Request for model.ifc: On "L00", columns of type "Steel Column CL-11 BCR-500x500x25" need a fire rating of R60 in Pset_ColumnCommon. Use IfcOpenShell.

First a look at what the model holds.

```python
import ifcopenshell
import ifcopenshell.util.element

model = ifcopenshell.open("model.ifc")
print(model.schema)
storey = next(s for s in model.by_type("IfcBuildingStorey") if s.Name == "L00")
columns = [e for e in ifcopenshell.util.element.get_decomposition(storey) if e.is_a("IfcColumn")]
seen = {}
for e in columns:
    element_type = ifcopenshell.util.element.get_type(e)
    key = (element_type.Name if element_type != e and element_type else None, ifcopenshell.util.element.get_pset(e, "Pset_ColumnCommon", "FireRating"))
    seen[key] = seen.get(key, 0) + 1
for (name, value), count in sorted(seen.items(), key=str):
    print(count, "x", name, "|", value)
```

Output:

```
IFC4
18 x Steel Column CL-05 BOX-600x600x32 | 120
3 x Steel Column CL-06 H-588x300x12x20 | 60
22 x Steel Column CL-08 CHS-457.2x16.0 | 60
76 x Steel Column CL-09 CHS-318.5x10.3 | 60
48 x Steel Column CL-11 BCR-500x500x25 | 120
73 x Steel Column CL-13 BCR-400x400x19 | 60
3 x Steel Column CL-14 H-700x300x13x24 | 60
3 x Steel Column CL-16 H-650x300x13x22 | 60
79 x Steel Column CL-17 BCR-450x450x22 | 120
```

```python
import ifcopenshell
import ifcopenshell.api.pset
import ifcopenshell.util.element

model = ifcopenshell.open("model.ifc")

storey = next(s for s in model.by_type("IfcBuildingStorey") if s.Name == "L00")
columns = [e for e in ifcopenshell.util.element.get_decomposition(storey) if e.is_a("IfcColumn")]

count = 0
for e in columns:
    element_type = ifcopenshell.util.element.get_type(e)
    if element_type in (None, e) or element_type.Name != "Steel Column CL-11 BCR-500x500x25":
        continue
    # add_pset returns the element's existing set when there is one.
    pset = ifcopenshell.api.pset.add_pset(model, product=e, name="Pset_ColumnCommon")
    ifcopenshell.api.pset.edit_pset(model, pset=pset, properties={"FireRating": "R60"})
    count += 1

print(count, "columns updated")

model.write("model_rev.ifc")
```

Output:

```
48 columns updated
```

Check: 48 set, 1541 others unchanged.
